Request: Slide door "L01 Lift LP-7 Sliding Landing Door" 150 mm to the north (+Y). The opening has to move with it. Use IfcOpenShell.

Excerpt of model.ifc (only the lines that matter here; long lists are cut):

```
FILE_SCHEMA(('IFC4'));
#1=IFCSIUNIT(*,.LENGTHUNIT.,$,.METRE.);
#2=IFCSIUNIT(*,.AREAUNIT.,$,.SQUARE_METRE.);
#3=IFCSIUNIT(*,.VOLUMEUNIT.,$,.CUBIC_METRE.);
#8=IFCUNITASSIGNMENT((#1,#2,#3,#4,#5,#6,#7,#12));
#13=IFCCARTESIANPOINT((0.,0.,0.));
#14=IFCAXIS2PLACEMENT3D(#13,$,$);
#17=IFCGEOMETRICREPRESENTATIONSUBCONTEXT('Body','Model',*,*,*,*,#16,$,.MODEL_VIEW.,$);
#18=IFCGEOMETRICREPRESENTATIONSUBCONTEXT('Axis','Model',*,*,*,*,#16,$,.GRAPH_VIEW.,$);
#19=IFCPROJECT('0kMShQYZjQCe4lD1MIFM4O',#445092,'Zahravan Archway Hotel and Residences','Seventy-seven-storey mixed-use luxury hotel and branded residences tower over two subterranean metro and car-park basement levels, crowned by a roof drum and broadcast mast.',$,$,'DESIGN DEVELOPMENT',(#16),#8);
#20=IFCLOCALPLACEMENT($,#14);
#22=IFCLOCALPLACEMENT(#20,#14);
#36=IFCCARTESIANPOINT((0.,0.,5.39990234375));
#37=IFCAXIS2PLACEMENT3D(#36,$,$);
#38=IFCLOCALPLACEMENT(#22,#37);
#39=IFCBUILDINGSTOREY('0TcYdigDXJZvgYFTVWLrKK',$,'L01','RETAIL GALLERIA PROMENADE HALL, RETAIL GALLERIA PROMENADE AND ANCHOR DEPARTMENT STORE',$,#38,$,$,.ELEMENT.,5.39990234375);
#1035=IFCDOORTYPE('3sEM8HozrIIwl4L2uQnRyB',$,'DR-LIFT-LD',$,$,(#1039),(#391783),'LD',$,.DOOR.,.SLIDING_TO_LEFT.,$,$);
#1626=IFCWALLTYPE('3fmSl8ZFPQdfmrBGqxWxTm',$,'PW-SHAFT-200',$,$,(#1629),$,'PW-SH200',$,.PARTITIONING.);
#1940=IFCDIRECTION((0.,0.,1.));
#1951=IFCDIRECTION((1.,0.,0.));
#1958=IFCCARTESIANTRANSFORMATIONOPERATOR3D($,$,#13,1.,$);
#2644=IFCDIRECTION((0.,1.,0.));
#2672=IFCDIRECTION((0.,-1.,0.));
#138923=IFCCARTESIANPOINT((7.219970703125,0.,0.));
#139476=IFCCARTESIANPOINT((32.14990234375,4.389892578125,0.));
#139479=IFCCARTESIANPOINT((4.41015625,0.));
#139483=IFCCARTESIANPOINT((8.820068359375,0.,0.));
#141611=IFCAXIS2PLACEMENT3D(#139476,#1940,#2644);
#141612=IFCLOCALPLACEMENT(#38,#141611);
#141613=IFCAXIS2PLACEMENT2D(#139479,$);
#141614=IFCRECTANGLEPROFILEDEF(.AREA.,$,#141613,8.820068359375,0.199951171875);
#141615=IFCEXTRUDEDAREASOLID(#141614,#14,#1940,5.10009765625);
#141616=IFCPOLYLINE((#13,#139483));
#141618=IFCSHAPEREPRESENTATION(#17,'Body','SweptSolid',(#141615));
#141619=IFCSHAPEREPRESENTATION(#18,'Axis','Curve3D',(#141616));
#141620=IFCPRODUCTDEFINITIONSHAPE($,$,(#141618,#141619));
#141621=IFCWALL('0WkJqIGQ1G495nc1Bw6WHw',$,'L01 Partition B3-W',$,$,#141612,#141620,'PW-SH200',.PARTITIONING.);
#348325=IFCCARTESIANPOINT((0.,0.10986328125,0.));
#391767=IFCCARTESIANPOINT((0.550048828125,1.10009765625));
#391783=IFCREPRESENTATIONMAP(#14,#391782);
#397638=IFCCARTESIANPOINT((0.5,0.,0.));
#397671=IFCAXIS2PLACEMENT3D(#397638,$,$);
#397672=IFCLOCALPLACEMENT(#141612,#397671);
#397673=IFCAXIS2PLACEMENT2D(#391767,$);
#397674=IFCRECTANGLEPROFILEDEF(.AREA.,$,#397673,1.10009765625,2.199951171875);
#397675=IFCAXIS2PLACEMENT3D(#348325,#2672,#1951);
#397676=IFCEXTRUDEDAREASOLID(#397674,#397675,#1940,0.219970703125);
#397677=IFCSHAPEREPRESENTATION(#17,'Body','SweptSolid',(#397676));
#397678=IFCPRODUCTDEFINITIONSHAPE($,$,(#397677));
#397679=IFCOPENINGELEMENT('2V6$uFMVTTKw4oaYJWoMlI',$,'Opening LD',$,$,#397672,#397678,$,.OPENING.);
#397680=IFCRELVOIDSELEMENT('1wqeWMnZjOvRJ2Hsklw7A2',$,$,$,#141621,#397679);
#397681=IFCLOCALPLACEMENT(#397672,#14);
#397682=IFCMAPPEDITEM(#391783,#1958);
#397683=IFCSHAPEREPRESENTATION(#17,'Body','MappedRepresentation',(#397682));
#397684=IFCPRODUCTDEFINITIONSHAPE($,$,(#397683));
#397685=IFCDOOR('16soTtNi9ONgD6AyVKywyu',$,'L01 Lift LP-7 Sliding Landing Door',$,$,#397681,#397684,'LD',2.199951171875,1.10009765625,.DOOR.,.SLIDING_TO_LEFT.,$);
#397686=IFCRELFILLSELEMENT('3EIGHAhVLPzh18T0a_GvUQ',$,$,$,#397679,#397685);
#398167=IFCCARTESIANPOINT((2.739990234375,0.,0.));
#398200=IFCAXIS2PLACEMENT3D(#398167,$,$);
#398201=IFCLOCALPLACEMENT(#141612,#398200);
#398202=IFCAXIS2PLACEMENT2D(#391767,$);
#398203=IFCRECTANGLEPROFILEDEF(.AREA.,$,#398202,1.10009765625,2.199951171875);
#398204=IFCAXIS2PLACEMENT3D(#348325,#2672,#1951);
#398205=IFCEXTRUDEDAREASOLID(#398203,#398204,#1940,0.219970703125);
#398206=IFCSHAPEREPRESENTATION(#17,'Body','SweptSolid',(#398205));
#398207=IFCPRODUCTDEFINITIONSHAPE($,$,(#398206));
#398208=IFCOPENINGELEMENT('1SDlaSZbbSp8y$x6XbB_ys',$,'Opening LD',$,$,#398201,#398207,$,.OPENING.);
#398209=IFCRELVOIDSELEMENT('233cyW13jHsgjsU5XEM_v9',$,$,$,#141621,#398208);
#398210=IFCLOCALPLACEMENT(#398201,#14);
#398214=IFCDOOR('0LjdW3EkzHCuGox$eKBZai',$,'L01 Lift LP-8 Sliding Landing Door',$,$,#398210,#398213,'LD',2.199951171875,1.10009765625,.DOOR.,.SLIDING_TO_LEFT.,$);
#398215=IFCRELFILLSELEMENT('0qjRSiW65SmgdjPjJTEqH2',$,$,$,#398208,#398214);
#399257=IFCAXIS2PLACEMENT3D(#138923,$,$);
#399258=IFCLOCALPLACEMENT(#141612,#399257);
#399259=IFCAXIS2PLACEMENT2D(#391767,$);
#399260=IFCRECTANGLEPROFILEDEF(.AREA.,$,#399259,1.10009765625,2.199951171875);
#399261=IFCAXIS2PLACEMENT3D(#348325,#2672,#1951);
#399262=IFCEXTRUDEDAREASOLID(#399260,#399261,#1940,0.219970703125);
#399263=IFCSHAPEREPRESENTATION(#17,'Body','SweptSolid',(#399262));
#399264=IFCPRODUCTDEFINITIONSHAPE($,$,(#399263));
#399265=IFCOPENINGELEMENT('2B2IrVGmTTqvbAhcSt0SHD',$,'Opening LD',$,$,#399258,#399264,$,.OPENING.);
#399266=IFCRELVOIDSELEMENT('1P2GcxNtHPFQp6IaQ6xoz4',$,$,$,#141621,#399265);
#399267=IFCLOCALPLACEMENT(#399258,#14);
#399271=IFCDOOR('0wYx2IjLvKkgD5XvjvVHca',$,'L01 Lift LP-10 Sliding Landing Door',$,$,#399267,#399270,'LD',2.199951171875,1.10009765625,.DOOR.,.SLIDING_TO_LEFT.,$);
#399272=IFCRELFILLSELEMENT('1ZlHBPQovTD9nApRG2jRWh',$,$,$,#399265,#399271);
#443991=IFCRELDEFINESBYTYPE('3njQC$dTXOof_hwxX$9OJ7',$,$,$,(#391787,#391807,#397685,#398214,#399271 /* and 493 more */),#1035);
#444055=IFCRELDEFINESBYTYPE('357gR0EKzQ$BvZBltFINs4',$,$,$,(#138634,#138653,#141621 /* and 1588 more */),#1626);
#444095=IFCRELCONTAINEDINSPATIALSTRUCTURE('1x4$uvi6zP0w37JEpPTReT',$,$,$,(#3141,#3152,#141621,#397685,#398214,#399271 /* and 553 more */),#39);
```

```python
import ifcopenshell
import ifcopenshell.api.geometry
import ifcopenshell.util.placement
import ifcopenshell.util.unit

model = ifcopenshell.open("model.ifc")
unit_scale = ifcopenshell.util.unit.calculate_unit_scale(model)

door = model.by_id(397685)
opening = door.FillsVoids[0].RelatingOpeningElement
wall = opening.VoidsElements[0].RelatingBuildingElement

wall_matrix = ifcopenshell.util.placement.get_local_placement(wall.ObjectPlacement)
shift = wall_matrix[:3, 0] * 0.15 / unit_scale
before = ifcopenshell.util.placement.get_local_placement(door.ObjectPlacement)[:3, 3].copy()

# The door is placed relative to its opening, so it follows when the opening moves.
matrix = ifcopenshell.util.placement.get_local_placement(opening.ObjectPlacement)
matrix[:3, 3] += shift
ifcopenshell.api.geometry.edit_object_placement(
    model, product=opening, matrix=matrix, is_si=False, should_transform_children=True
)

after = ifcopenshell.util.placement.get_local_placement(door.ObjectPlacement)[:3, 3]
print("door moved by", (after - before).round(3) + 0.0)

model.write("model_v2.ifc")
```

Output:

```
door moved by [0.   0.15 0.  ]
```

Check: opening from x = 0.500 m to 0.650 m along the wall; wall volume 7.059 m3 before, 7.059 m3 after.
